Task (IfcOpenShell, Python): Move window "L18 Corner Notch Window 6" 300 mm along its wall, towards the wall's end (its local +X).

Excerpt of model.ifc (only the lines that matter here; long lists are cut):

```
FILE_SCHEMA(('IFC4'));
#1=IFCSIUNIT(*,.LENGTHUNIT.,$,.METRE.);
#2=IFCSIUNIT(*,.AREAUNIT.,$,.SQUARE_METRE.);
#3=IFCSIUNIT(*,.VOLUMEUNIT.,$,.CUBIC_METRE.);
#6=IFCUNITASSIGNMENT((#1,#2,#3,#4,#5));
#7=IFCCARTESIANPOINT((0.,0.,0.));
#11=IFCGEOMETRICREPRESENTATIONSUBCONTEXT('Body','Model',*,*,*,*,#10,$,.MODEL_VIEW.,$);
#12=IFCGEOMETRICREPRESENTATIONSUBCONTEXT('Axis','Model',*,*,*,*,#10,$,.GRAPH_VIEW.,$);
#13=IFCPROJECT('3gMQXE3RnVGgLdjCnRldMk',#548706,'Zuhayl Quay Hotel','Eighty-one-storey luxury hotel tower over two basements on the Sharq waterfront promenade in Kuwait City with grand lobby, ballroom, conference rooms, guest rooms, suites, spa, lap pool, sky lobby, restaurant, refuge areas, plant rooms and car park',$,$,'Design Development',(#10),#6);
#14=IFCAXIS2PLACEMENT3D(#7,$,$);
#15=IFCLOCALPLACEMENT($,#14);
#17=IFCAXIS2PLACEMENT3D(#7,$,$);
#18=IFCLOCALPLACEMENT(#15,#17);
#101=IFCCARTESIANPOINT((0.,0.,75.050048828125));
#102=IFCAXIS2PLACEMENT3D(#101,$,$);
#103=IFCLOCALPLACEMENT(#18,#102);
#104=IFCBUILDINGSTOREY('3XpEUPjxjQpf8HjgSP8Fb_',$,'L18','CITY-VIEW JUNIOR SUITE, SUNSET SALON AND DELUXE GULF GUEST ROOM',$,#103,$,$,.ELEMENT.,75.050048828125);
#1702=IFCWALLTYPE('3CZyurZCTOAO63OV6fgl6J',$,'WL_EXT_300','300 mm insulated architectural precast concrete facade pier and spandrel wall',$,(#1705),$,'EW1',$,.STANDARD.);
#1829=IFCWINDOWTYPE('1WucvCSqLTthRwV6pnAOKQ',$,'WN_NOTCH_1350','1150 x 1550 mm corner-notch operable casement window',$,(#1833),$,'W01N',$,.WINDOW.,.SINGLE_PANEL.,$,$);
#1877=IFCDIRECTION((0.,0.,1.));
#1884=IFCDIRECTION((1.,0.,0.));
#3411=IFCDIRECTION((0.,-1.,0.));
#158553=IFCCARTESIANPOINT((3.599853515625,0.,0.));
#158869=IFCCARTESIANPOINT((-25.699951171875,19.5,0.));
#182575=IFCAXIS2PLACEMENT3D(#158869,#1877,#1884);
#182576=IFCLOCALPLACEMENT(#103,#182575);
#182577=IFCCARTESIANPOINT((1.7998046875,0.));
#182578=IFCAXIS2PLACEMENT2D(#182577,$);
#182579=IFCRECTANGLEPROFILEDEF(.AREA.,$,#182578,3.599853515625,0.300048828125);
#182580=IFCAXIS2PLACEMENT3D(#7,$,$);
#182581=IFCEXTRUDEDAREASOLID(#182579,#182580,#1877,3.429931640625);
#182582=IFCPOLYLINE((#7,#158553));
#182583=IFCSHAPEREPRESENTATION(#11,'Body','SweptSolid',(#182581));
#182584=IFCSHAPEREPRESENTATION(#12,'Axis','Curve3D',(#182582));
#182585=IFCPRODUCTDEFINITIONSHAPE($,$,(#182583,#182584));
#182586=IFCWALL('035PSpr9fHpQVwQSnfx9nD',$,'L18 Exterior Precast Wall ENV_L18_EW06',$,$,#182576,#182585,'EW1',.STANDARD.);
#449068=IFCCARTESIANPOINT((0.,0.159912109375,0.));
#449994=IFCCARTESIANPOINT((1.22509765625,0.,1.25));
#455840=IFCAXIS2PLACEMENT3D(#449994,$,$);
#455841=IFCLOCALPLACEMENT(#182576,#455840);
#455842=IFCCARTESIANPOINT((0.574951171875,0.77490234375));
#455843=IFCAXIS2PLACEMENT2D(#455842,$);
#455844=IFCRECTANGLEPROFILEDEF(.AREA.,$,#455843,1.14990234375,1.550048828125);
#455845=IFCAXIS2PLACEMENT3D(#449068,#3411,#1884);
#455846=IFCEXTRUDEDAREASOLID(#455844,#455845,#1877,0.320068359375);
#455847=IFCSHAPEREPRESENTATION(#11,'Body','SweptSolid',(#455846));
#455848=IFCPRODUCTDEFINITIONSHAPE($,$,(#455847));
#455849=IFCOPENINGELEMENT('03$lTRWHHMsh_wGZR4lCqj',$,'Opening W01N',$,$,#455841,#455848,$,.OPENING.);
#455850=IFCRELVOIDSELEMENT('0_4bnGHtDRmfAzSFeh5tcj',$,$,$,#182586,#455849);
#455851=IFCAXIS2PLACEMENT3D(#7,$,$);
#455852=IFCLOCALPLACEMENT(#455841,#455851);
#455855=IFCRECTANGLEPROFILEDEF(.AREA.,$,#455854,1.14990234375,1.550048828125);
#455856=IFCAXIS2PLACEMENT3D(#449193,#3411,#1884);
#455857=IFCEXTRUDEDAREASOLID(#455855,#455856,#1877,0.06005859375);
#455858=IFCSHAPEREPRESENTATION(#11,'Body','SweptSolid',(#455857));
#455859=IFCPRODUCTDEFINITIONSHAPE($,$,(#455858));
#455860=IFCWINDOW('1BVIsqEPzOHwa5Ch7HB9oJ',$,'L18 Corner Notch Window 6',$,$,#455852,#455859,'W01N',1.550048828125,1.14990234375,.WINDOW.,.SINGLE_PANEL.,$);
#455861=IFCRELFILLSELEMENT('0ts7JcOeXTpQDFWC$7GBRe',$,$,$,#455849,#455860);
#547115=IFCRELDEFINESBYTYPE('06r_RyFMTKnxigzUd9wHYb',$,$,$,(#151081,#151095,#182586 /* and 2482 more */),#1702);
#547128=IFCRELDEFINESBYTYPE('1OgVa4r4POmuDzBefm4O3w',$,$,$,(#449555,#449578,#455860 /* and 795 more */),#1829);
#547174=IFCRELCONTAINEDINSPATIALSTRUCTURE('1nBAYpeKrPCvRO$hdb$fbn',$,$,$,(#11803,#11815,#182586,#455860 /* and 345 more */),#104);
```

```python
import ifcopenshell
import ifcopenshell.api.geometry
import ifcopenshell.util.placement
import ifcopenshell.util.unit

model = ifcopenshell.open("model.ifc")
unit_scale = ifcopenshell.util.unit.calculate_unit_scale(model)

window = model.by_guid("1BVIsqEPzOHwa5Ch7HB9oJ")
opening = window.FillsVoids[0].RelatingOpeningElement
wall = opening.VoidsElements[0].RelatingBuildingElement

wall_matrix = ifcopenshell.util.placement.get_local_placement(wall.ObjectPlacement)
shift = wall_matrix[:3, 0] * 0.3 / unit_scale
before = ifcopenshell.util.placement.get_local_placement(window.ObjectPlacement)[:3, 3].copy()

# The window is placed relative to its opening, so it follows when the opening moves.
matrix = ifcopenshell.util.placement.get_local_placement(opening.ObjectPlacement)
matrix[:3, 3] += shift
ifcopenshell.api.geometry.edit_object_placement(
    model, product=opening, matrix=matrix, is_si=False, should_transform_children=True
)

after = ifcopenshell.util.placement.get_local_placement(window.ObjectPlacement)[:3, 3]
print("window moved by", (after - before).round(3) + 0.0)

model.write("model-out.ifc")
```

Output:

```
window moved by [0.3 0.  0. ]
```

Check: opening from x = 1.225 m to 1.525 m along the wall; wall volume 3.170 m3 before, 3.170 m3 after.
